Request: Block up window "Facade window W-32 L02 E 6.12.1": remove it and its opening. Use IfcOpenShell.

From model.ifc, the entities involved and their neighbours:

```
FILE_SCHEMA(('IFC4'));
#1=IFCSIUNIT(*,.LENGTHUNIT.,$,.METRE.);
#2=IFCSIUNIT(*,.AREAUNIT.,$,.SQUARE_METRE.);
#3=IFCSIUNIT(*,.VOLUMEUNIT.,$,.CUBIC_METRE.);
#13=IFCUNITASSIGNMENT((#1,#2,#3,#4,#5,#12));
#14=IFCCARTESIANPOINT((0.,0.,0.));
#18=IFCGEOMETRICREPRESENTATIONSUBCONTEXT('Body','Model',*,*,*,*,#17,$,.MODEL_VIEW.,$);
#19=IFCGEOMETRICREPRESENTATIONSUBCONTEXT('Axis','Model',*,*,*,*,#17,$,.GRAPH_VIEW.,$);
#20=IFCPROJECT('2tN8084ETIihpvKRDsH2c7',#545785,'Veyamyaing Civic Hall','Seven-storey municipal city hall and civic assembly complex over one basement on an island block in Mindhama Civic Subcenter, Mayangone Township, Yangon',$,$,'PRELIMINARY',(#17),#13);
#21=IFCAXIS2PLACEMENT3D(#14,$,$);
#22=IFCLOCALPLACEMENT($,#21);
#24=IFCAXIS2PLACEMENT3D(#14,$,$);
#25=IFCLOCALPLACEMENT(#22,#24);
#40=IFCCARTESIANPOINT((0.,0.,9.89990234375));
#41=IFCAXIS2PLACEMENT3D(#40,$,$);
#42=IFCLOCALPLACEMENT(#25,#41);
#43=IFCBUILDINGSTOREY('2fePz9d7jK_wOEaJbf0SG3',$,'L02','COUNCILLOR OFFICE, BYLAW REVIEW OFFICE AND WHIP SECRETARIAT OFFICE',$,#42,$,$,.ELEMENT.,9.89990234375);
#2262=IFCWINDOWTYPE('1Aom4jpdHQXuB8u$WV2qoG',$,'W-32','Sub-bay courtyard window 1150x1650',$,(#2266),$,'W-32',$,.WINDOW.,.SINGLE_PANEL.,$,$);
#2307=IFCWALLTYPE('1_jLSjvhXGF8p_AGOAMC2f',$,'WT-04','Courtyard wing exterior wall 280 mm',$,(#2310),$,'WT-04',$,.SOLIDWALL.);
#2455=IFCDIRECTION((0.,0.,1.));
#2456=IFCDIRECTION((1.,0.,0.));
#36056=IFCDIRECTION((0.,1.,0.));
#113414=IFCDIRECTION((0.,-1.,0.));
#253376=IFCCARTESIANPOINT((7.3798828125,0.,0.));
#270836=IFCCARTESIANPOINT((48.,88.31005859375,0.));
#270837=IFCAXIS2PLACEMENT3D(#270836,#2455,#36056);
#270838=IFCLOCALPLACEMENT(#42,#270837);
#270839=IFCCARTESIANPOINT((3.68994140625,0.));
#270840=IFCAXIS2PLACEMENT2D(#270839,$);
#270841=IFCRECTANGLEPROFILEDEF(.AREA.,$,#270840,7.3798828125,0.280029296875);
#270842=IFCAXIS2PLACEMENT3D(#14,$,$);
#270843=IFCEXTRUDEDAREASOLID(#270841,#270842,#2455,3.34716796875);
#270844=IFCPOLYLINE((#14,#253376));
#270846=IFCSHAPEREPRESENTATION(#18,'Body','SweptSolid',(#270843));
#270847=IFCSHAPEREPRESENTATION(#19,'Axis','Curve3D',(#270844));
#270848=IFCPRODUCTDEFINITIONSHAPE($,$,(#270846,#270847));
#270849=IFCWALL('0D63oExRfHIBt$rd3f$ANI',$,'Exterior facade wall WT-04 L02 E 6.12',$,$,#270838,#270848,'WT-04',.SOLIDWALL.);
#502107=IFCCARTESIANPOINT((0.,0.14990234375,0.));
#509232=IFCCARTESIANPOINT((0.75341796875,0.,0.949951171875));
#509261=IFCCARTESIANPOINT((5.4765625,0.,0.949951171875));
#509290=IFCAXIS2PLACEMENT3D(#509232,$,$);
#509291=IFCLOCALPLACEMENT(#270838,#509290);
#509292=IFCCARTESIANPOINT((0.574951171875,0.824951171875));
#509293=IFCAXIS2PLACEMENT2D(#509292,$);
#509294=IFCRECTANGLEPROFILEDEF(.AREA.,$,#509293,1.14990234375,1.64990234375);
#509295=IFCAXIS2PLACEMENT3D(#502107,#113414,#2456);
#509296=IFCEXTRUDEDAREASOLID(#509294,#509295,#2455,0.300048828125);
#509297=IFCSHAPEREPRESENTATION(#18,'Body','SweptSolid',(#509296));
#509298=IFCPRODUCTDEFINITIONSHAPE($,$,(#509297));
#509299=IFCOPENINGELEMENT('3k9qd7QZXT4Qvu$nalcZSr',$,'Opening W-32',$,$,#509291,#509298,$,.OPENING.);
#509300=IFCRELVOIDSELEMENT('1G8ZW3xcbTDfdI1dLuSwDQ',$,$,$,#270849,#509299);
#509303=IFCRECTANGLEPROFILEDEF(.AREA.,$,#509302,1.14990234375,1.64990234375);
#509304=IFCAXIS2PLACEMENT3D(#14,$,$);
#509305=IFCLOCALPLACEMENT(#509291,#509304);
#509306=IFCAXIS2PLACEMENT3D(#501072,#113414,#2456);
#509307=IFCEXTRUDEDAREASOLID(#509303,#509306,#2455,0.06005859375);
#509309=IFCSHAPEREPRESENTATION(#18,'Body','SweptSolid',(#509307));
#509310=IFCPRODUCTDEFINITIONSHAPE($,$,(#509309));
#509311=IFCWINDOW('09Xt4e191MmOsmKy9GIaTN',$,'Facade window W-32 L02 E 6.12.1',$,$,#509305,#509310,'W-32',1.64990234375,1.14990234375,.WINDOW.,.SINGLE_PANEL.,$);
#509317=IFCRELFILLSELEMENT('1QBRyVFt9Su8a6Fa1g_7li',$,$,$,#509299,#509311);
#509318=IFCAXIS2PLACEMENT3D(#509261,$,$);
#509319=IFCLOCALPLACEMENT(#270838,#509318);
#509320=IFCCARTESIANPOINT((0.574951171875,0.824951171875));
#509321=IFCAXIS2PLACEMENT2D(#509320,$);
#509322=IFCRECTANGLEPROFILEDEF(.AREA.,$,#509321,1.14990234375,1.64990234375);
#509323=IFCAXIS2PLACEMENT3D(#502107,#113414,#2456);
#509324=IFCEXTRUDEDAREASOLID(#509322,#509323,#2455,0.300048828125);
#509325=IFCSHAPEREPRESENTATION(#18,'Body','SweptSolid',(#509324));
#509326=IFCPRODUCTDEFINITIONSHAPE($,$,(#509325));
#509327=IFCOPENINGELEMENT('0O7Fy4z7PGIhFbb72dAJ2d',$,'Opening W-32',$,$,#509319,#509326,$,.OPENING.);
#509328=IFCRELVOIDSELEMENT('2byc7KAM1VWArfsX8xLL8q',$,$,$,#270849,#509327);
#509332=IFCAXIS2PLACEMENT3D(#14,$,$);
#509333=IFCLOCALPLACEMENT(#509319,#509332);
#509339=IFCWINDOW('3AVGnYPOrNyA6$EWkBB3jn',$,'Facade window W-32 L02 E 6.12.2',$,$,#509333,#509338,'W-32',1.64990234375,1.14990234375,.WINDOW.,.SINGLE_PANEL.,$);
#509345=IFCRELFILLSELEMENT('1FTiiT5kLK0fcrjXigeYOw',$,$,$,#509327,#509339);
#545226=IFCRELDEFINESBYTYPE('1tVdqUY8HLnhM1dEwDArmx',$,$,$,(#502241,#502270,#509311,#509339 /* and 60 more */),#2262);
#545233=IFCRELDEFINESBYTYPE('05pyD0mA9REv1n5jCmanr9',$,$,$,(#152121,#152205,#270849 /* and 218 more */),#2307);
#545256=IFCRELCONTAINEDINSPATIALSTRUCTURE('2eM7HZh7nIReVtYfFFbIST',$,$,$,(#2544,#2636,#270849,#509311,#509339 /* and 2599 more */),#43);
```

```python
import ifcopenshell
import ifcopenshell.api.feature
import ifcopenshell.api.root
import ifcopenshell.geom
import ifcopenshell.util.shape

model = ifcopenshell.open("model.ifc")
settings = ifcopenshell.geom.settings()


def volume(element):
    """Net volume in cubic metres, openings subtracted."""
    shape = ifcopenshell.geom.create_shape(settings, element)
    return ifcopenshell.util.shape.get_volume(shape.geometry)


window = model.by_id(509311)
opening = window.FillsVoids[0].RelatingOpeningElement
wall = opening.VoidsElements[0].RelatingBuildingElement
before = volume(wall)

ifcopenshell.api.root.remove_product(model, product=window)
ifcopenshell.api.feature.remove_feature(model, feature=opening)

after = volume(wall)

print(f"wall volume {before:.3f} -> {after:.3f} m3")

model.write("model_updated.ifc")
```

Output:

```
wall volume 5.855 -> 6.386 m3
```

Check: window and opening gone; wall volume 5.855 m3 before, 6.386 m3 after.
